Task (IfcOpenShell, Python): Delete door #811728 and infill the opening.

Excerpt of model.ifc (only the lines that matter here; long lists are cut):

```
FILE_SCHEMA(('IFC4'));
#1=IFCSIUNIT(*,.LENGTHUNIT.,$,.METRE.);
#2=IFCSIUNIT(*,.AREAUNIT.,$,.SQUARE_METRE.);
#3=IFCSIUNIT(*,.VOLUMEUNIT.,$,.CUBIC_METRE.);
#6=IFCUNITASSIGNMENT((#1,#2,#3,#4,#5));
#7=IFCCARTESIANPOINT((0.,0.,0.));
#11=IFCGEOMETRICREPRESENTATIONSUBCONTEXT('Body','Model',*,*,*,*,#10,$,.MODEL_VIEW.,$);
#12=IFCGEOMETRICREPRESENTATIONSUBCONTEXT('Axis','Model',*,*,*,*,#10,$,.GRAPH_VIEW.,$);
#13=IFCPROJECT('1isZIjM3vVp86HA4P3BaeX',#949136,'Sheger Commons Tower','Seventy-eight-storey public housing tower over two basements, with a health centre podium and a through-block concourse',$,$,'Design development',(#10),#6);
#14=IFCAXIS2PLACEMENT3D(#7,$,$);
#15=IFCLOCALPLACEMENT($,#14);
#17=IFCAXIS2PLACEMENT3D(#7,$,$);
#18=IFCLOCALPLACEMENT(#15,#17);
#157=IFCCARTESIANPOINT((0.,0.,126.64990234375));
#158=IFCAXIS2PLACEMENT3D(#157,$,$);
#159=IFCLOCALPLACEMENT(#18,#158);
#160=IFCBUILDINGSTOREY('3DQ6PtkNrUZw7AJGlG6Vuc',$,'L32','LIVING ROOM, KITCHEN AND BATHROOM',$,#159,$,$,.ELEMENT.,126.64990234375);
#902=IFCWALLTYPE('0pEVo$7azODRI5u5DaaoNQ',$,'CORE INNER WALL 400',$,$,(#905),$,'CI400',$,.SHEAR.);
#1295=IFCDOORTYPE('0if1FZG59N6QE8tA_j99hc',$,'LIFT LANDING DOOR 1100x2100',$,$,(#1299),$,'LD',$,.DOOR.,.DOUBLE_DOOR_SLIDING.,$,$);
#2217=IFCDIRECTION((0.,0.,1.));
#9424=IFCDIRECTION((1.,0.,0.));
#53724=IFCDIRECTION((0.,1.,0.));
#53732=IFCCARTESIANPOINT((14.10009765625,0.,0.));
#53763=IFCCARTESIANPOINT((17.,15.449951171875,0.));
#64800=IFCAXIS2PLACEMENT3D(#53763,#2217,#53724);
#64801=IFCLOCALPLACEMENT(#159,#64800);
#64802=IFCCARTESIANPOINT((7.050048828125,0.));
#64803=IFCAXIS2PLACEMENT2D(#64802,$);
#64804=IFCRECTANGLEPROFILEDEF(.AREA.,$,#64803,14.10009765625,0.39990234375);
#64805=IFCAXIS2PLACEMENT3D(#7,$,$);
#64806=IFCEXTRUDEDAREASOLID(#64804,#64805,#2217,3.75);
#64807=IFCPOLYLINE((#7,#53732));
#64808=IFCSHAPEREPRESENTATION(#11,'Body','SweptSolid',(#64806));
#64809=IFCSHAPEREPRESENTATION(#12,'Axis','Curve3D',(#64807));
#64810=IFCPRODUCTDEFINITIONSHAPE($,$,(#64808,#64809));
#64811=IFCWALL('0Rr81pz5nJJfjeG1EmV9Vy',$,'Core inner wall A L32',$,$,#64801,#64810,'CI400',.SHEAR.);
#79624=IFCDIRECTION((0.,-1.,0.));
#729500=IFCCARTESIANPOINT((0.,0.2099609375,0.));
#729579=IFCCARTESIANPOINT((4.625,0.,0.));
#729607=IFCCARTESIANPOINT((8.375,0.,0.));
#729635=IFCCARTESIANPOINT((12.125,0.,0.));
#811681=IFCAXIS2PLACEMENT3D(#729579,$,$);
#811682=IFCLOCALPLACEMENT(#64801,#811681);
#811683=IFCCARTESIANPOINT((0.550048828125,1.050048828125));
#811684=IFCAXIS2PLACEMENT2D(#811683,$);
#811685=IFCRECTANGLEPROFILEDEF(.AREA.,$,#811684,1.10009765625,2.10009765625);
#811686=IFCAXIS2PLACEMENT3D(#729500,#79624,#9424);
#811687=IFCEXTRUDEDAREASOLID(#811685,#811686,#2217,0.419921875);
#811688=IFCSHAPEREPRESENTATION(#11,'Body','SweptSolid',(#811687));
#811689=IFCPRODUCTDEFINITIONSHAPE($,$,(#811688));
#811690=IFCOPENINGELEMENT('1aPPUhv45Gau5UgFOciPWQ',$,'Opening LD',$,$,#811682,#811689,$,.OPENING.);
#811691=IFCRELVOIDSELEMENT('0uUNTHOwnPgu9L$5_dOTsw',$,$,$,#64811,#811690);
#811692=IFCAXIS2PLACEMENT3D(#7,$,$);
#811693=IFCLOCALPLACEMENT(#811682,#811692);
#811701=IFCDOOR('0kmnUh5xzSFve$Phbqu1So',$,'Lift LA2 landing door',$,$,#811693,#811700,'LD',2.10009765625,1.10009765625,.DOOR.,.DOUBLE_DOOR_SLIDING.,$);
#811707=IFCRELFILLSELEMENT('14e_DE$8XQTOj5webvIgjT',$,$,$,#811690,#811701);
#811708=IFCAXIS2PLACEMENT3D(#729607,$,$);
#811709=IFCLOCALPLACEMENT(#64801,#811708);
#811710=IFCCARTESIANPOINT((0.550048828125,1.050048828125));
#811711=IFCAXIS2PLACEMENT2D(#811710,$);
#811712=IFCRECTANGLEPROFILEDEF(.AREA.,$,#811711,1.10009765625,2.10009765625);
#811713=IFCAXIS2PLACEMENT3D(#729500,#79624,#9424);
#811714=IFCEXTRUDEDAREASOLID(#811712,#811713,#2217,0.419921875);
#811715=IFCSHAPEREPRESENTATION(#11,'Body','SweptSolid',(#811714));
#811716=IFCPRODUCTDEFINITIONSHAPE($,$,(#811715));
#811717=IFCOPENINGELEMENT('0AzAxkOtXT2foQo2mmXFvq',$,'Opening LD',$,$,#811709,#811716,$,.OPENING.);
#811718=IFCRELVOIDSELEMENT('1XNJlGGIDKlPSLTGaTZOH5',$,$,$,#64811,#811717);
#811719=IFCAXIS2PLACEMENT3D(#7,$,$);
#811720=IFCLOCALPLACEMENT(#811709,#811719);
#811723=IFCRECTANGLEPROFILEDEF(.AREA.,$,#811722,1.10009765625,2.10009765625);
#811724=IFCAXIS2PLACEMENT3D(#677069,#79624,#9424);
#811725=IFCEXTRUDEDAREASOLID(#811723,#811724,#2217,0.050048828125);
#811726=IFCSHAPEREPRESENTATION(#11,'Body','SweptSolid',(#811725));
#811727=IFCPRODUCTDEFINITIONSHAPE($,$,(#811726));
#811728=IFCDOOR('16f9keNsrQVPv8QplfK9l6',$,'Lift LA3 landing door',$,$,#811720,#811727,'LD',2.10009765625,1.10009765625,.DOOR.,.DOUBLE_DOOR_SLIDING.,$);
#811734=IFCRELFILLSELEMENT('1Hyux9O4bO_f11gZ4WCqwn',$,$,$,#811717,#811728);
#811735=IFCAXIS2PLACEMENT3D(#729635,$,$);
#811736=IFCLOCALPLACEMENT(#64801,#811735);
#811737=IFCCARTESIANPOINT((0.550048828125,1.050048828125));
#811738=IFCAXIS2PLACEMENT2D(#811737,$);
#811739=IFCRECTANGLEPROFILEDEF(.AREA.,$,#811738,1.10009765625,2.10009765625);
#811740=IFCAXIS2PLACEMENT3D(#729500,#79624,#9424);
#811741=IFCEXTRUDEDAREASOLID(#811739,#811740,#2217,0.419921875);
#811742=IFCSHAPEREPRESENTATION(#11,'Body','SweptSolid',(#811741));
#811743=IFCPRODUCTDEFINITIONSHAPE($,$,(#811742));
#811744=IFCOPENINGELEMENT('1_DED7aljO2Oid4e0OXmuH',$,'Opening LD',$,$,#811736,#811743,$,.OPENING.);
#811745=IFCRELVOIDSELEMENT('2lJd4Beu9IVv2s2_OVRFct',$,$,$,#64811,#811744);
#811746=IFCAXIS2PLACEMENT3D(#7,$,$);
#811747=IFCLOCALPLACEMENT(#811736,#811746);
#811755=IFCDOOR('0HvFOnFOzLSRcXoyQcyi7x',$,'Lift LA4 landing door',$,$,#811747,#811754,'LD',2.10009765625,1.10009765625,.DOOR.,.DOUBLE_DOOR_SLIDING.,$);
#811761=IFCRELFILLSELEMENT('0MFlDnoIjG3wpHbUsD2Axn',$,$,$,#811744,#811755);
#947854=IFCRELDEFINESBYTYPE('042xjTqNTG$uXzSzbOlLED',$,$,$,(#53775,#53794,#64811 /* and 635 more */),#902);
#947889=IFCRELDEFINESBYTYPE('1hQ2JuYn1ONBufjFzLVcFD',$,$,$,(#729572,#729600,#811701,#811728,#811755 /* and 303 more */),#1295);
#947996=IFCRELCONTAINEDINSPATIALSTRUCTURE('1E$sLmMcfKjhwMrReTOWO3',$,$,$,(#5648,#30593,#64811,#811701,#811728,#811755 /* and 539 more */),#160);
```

```python
import ifcopenshell
import ifcopenshell.api.feature
import ifcopenshell.api.root
import ifcopenshell.geom
import ifcopenshell.util.shape

model = ifcopenshell.open("model.ifc")
settings = ifcopenshell.geom.settings()


def volume(element):
    """Net volume in cubic metres, openings subtracted."""
    shape = ifcopenshell.geom.create_shape(settings, element)
    return ifcopenshell.util.shape.get_volume(shape.geometry)


door = model.by_id(811728)
opening = door.FillsVoids[0].RelatingOpeningElement
wall = opening.VoidsElements[0].RelatingBuildingElement
before = volume(wall)

ifcopenshell.api.root.remove_product(model, product=door)
ifcopenshell.api.feature.remove_feature(model, feature=opening)

after = volume(wall)

print(f"wall volume {before:.3f} -> {after:.3f} m3")

model.write("model-out.ifc")
```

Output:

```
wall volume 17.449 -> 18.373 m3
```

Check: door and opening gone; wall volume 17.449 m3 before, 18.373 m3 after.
